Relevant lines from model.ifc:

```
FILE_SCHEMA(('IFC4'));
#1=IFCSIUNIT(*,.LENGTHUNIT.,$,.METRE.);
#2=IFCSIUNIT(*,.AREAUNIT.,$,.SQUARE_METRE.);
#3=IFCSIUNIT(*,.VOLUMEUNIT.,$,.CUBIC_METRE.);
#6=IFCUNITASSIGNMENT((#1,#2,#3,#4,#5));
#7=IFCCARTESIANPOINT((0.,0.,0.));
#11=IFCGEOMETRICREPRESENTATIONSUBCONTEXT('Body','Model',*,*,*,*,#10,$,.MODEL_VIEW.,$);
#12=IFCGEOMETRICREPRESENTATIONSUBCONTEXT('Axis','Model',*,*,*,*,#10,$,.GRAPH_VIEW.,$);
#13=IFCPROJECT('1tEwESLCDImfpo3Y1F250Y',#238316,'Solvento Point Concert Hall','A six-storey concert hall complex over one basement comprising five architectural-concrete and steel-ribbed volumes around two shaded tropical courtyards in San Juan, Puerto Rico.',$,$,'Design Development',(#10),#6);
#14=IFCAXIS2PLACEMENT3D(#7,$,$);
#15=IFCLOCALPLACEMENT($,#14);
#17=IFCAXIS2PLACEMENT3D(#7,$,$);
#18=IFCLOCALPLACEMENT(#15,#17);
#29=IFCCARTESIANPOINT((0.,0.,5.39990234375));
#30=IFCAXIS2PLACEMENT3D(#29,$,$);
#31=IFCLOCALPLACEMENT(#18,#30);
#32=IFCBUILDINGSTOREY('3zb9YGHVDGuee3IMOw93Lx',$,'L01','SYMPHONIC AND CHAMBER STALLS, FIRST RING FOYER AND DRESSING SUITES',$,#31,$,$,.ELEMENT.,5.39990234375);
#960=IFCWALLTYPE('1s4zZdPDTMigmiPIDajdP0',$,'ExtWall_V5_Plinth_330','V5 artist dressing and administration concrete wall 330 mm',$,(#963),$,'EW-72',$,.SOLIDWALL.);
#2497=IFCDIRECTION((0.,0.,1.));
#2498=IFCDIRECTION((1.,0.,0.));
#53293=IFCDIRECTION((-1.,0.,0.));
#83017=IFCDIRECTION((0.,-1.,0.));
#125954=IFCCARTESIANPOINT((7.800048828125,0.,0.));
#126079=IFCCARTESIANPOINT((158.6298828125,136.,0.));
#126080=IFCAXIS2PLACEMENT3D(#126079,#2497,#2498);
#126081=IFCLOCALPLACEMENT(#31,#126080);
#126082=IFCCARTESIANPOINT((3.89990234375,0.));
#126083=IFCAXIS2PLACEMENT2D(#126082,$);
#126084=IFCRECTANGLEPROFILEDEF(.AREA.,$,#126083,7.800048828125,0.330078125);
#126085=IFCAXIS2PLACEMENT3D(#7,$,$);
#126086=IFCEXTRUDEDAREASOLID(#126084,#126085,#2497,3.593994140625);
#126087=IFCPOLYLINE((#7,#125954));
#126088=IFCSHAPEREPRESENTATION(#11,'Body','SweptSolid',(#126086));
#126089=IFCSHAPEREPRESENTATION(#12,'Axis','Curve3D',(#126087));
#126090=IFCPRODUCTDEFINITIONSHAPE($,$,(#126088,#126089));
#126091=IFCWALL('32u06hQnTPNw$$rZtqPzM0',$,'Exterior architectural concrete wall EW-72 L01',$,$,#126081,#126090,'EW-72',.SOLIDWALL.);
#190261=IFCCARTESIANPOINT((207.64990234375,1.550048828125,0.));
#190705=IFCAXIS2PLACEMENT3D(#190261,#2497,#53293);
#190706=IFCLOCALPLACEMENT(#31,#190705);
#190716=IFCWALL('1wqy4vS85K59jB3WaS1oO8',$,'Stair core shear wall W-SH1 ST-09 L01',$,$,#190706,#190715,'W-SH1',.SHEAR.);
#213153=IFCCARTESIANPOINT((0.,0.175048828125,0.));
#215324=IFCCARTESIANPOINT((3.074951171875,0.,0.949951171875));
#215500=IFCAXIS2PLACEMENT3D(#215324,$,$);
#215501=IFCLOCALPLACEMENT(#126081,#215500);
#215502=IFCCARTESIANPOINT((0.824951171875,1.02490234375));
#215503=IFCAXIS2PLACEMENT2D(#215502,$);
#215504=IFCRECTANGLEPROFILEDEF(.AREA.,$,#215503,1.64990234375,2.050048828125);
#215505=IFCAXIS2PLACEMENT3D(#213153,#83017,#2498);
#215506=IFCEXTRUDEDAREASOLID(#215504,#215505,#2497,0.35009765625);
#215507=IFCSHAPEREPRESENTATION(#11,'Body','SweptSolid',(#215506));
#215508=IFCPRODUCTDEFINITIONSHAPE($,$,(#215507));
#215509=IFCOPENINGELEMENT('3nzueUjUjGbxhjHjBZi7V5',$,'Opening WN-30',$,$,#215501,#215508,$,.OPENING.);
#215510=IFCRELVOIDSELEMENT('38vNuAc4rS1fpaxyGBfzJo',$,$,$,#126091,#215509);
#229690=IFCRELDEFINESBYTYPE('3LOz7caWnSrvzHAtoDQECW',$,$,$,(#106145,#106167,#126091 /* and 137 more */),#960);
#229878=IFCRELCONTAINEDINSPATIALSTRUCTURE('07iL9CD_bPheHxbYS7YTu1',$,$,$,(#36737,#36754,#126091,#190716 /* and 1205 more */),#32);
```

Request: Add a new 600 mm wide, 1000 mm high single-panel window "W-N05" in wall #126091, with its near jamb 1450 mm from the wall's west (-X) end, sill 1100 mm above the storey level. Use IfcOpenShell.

```python
import numpy as np
import ifcopenshell
import ifcopenshell.api.feature
import ifcopenshell.api.geometry
import ifcopenshell.api.root
import ifcopenshell.api.spatial
import ifcopenshell.geom
import ifcopenshell.util.element
import ifcopenshell.util.placement
import ifcopenshell.util.representation
import ifcopenshell.util.shape
import ifcopenshell.util.unit

model = ifcopenshell.open("model.ifc")
unit_scale = ifcopenshell.util.unit.calculate_unit_scale(model)
settings = ifcopenshell.geom.settings()


def volume(element):
    """Net volume in cubic metres, openings subtracted."""
    shape = ifcopenshell.geom.create_shape(settings, element)
    return ifcopenshell.util.shape.get_volume(shape.geometry)


wall = model.by_guid("32u06hQnTPNw$$rZtqPzM0")
storey = ifcopenshell.util.element.get_container(wall, ifc_class="IfcBuildingStorey")
context = ifcopenshell.util.representation.get_context(model, "Model", "Body", "MODEL_VIEW")
before = volume(wall)

width, height, from_end, sill = 0.6, 1, 1.45, 1.1  # metres

# The wall runs along its own X axis, and the end named is its -X end.
wall_shape = ifcopenshell.geom.create_shape(settings, wall)
x, y, z = ifcopenshell.util.shape.get_vertices(wall_shape.geometry).T
start = x.min() + from_end
face, thickness = float(y.min()), float(y.max() - y.min())
wall_matrix = ifcopenshell.util.placement.get_local_placement(wall.ObjectPlacement)
level = ifcopenshell.util.placement.get_local_placement(storey.ObjectPlacement)[2, 3]


def in_wall(x, y):
    """Placement at x, y metres in the wall's axes, at sill height."""
    matrix = wall_matrix.copy()
    matrix[:, 3] = wall_matrix @ np.array([x / unit_scale, y / unit_scale, 0.0, 1.0])
    matrix[2, 3] = level + sill / unit_scale
    return matrix


# Opening: a box that overshoots both wall faces by 50 mm.
opening = ifcopenshell.api.root.create_entity(model, ifc_class="IfcOpeningElement", predefined_type="OPENING")
box = ifcopenshell.api.geometry.add_wall_representation(
    model, context=context, length=width, height=height, thickness=thickness + 0.1
)
ifcopenshell.api.geometry.assign_representation(model, product=opening, representation=box)
ifcopenshell.api.geometry.edit_object_placement(model, product=opening, matrix=in_wall(start, face - 0.05), is_si=False)
ifcopenshell.api.feature.add_feature(model, feature=opening, element=wall)

window = ifcopenshell.api.root.create_entity(model, ifc_class="IfcWindow", name="W-N05", predefined_type="WINDOW")
window.OverallWidth, window.OverallHeight = width / unit_scale, height / unit_scale
window.PartitioningType = "SINGLE_PANEL"
body = ifcopenshell.api.geometry.add_window_representation(
    model,
    context=context,
    overall_width=window.OverallWidth,
    overall_height=window.OverallHeight,
    partition_type="SINGLE_PANEL",
)
ifcopenshell.api.geometry.assign_representation(model, product=window, representation=body)
ifcopenshell.api.spatial.assign_container(model, products=[window], relating_structure=storey)
ifcopenshell.api.feature.add_filling(model, opening=opening, element=window)

# Centre the window in the wall's thickness.
ifcopenshell.api.geometry.edit_object_placement(model, product=window, matrix=in_wall(start, face), is_si=False)
window_shape = ifcopenshell.geom.create_shape(settings, window)
depth = ifcopenshell.util.shape.get_vertices(window_shape.geometry)[:, 1]
offset = face + thickness / 2 - (depth.min() + depth.max()) / 2
ifcopenshell.api.geometry.edit_object_placement(model, product=window, matrix=in_wall(start, offset), is_si=False)

after = volume(wall)

print(f"wall volume {before:.3f} -> {after:.3f} m3")

model.write("model_updated.ifc")
```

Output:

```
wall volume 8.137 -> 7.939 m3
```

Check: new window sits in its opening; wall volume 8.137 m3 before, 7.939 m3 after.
